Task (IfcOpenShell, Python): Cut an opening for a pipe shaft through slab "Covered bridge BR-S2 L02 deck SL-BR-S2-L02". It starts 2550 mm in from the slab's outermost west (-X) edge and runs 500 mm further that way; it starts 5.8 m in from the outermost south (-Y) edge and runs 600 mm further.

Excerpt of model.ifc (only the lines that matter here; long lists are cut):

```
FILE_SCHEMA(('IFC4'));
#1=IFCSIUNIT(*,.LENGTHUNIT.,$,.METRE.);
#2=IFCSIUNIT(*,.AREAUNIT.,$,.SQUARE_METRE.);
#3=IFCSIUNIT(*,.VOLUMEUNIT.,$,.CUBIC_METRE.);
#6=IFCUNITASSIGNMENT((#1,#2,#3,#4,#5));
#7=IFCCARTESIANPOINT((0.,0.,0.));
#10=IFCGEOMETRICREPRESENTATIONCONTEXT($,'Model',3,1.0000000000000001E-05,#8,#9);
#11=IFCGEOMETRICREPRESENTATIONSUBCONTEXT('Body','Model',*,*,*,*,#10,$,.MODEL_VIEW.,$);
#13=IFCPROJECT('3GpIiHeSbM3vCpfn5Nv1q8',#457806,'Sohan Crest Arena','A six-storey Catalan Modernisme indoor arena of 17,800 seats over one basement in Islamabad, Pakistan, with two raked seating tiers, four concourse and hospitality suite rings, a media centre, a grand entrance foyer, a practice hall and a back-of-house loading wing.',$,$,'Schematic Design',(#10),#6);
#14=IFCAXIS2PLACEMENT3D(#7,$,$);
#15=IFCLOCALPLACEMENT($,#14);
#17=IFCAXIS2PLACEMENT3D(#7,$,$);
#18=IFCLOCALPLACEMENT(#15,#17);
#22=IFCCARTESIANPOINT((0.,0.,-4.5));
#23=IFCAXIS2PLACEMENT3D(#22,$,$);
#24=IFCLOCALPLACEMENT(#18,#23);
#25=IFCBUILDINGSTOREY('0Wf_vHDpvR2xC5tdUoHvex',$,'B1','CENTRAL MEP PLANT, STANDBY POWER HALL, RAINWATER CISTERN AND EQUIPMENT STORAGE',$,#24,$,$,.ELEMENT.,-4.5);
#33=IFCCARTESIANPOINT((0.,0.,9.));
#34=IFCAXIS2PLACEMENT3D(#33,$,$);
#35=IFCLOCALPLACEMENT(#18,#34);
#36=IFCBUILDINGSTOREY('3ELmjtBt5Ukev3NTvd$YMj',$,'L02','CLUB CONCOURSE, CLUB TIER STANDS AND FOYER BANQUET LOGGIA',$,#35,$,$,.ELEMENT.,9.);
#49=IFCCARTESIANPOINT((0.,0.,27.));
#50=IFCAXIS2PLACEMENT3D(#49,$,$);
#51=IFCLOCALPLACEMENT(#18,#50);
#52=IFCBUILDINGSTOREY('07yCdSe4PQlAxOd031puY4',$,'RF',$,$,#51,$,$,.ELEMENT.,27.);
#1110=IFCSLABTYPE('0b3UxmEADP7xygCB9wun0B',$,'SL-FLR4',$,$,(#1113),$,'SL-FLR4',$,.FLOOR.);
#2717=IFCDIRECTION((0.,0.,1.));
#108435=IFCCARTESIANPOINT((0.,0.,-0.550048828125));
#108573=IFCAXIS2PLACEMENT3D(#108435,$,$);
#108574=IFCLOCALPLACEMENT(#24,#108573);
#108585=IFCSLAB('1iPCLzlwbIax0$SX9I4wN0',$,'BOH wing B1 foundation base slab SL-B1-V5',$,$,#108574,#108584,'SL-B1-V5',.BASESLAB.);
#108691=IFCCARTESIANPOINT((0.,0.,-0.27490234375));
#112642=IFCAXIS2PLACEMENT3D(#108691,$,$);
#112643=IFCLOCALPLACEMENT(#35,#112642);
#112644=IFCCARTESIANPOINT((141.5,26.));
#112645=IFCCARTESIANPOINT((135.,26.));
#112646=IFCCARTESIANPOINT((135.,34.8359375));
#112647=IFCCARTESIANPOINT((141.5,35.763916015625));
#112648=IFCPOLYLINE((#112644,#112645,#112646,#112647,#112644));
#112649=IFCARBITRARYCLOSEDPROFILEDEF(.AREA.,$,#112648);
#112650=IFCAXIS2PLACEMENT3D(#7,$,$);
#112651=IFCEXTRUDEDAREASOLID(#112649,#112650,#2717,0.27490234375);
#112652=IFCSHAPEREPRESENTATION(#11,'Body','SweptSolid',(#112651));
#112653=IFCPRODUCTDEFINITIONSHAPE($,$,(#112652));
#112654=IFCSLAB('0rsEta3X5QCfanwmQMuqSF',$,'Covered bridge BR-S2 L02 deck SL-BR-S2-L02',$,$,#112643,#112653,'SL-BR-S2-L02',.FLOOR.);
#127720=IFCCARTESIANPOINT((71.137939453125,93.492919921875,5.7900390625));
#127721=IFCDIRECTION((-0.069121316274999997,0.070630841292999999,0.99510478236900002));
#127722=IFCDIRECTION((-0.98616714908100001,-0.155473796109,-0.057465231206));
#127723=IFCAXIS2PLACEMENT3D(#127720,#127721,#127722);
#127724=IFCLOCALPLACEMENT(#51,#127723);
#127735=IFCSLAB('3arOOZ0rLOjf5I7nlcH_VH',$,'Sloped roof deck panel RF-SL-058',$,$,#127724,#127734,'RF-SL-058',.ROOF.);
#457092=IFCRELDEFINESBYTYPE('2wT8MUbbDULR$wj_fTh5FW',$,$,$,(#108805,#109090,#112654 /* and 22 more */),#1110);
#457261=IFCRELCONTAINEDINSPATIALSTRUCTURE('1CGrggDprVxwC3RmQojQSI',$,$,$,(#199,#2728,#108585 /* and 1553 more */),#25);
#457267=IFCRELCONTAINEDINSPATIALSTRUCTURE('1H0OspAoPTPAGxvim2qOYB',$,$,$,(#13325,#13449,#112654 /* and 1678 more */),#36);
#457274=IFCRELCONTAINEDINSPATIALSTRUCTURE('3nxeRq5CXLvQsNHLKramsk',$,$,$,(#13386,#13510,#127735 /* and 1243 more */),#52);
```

```python
import numpy as np
import ifcopenshell
import ifcopenshell.api.feature
import ifcopenshell.api.geometry
import ifcopenshell.api.root
import ifcopenshell.geom
import ifcopenshell.util.placement
import ifcopenshell.util.representation
import ifcopenshell.util.shape
import ifcopenshell.util.unit

model = ifcopenshell.open("model.ifc")
unit_scale = ifcopenshell.util.unit.calculate_unit_scale(model)
settings = ifcopenshell.geom.settings()


def volume(element):
    """Net volume in cubic metres, openings subtracted."""
    shape = ifcopenshell.geom.create_shape(settings, element)
    return ifcopenshell.util.shape.get_volume(shape.geometry)


slab = model.by_guid("0rsEta3X5QCfanwmQMuqSF")
before = volume(slab)

# Extent in the slab's own axes, in metres. The edges named are its -X and -Y sides.
slab_shape = ifcopenshell.geom.create_shape(settings, slab)
vertices = ifcopenshell.util.shape.get_vertices(slab_shape.geometry)
x_min, y_min, bottom = vertices.min(axis=0)
top = vertices[:, 2].max()

opening = ifcopenshell.api.root.create_entity(model, ifc_class="IfcOpeningElement", name="Pipe shaft opening", predefined_type="OPENING")
context = ifcopenshell.util.representation.get_context(model, "Model", "Body", "MODEL_VIEW")
width, depth = 0.5, 0.6
outline = [(0.0, 0.0), (width, 0.0), (width, depth), (0.0, depth), (0.0, 0.0)]
# Overshoot both faces by 50 mm so the cut is clean.
shape = ifcopenshell.api.geometry.add_slab_representation(
    model, context=context, depth=top - bottom + 0.1, polyline=outline
)
ifcopenshell.api.geometry.assign_representation(model, product=opening, representation=shape)

matrix = ifcopenshell.util.placement.get_local_placement(slab.ObjectPlacement)
matrix[:, 3] = matrix @ np.append(np.array([x_min + 2.55, y_min + 5.8, bottom - 0.05]) / unit_scale, 1.0)
ifcopenshell.api.geometry.edit_object_placement(model, product=opening, matrix=matrix, is_si=False)
ifcopenshell.api.feature.add_feature(model, feature=opening, element=slab)

after = volume(slab)

print(f"slab volume {before:.3f} -> {after:.3f} m3")

model.write("model-out.ifc")
```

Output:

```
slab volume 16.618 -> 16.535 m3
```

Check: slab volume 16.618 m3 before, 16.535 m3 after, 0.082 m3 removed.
